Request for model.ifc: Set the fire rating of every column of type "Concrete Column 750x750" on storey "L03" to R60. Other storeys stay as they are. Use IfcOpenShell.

First a look at what the model holds.

```python
import ifcopenshell
import ifcopenshell.util.element

model = ifcopenshell.open("model.ifc")
print(model.schema)
storey = next(s for s in model.by_type("IfcBuildingStorey") if s.Name == "L03")
columns = [e for e in ifcopenshell.util.element.get_decomposition(storey) if e.is_a("IfcColumn")]
seen = {}
for e in columns:
    element_type = ifcopenshell.util.element.get_type(e)
    key = (element_type.Name if element_type != e and element_type else None, ifcopenshell.util.element.get_pset(e, "Pset_ColumnCommon", "FireRating"))
    seen[key] = seen.get(key, 0) + 1
for (name, value), count in sorted(seen.items(), key=str):
    print(count, "x", name, "|", value)
```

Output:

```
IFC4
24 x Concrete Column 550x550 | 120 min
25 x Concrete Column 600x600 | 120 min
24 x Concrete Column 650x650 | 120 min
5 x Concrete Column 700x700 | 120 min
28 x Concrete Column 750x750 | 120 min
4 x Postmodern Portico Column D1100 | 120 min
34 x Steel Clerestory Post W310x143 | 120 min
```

```python
import ifcopenshell
import ifcopenshell.api.pset
import ifcopenshell.util.element

model = ifcopenshell.open("model.ifc")

storey = next(s for s in model.by_type("IfcBuildingStorey") if s.Name == "L03")
columns = [e for e in ifcopenshell.util.element.get_decomposition(storey) if e.is_a("IfcColumn")]

count = 0
for e in columns:
    element_type = ifcopenshell.util.element.get_type(e)
    if element_type in (None, e) or element_type.Name != "Concrete Column 750x750":
        continue
    # add_pset returns the element's existing set when there is one.
    pset = ifcopenshell.api.pset.add_pset(model, product=e, name="Pset_ColumnCommon")
    ifcopenshell.api.pset.edit_pset(model, pset=pset, properties={"FireRating": "R60"})
    count += 1

print(count, "columns updated")

model.write("model_v2.ifc")
```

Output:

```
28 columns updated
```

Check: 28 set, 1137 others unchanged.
